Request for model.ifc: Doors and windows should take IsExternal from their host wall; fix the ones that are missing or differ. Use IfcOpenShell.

First a look at what the model holds.

```python
import ifcopenshell
import ifcopenshell.util.element

model = ifcopenshell.open("model.ifc")
print(model.schema)
seen = {}
for e in model.by_type("IfcDoor") + model.by_type("IfcWindow"):
    if not e.FillsVoids:
        continue
    host = e.FillsVoids[0].RelatingOpeningElement.VoidsElements[0].RelatingBuildingElement
    own = ifcopenshell.util.element.get_pset(e, f"Pset_{e.is_a()[3:].removesuffix('StandardCase')}Common", "IsExternal")
    wall = ifcopenshell.util.element.get_pset(host, "Pset_WallCommon", "IsExternal")
    seen[e.is_a(), own, wall] = seen.get((e.is_a(), own, wall), 0) + 1
for (cls, own, wall), count in sorted(seen.items(), key=str):
    print(count, cls, "IsExternal:", own, "| host wall:", wall)
```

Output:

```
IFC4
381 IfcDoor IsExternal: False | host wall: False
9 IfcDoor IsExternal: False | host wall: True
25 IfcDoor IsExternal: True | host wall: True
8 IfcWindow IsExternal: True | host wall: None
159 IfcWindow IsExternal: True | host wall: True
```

```python
import ifcopenshell
import ifcopenshell.api.pset
import ifcopenshell.util.element

model = ifcopenshell.open("model.ifc")

count = 0
for ifc_class, pset_name in (("IfcDoor", "Pset_DoorCommon"), ("IfcWindow", "Pset_WindowCommon")):
    for e in model.by_type(ifc_class):
        if not e.FillsVoids:
            continue
        host = e.FillsVoids[0].RelatingOpeningElement.VoidsElements[0].RelatingBuildingElement
        external = ifcopenshell.util.element.get_pset(host, "Pset_WallCommon", "IsExternal")
        if external is None or ifcopenshell.util.element.get_pset(e, pset_name, "IsExternal") == external:
            continue
        pset = ifcopenshell.api.pset.add_pset(model, product=e, name=pset_name)
        ifcopenshell.api.pset.edit_pset(model, pset=pset, properties={"IsExternal": external})
        count += 1

print(count, "updated")

model.write("model_edited.ifc")
```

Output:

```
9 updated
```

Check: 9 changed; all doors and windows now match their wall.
